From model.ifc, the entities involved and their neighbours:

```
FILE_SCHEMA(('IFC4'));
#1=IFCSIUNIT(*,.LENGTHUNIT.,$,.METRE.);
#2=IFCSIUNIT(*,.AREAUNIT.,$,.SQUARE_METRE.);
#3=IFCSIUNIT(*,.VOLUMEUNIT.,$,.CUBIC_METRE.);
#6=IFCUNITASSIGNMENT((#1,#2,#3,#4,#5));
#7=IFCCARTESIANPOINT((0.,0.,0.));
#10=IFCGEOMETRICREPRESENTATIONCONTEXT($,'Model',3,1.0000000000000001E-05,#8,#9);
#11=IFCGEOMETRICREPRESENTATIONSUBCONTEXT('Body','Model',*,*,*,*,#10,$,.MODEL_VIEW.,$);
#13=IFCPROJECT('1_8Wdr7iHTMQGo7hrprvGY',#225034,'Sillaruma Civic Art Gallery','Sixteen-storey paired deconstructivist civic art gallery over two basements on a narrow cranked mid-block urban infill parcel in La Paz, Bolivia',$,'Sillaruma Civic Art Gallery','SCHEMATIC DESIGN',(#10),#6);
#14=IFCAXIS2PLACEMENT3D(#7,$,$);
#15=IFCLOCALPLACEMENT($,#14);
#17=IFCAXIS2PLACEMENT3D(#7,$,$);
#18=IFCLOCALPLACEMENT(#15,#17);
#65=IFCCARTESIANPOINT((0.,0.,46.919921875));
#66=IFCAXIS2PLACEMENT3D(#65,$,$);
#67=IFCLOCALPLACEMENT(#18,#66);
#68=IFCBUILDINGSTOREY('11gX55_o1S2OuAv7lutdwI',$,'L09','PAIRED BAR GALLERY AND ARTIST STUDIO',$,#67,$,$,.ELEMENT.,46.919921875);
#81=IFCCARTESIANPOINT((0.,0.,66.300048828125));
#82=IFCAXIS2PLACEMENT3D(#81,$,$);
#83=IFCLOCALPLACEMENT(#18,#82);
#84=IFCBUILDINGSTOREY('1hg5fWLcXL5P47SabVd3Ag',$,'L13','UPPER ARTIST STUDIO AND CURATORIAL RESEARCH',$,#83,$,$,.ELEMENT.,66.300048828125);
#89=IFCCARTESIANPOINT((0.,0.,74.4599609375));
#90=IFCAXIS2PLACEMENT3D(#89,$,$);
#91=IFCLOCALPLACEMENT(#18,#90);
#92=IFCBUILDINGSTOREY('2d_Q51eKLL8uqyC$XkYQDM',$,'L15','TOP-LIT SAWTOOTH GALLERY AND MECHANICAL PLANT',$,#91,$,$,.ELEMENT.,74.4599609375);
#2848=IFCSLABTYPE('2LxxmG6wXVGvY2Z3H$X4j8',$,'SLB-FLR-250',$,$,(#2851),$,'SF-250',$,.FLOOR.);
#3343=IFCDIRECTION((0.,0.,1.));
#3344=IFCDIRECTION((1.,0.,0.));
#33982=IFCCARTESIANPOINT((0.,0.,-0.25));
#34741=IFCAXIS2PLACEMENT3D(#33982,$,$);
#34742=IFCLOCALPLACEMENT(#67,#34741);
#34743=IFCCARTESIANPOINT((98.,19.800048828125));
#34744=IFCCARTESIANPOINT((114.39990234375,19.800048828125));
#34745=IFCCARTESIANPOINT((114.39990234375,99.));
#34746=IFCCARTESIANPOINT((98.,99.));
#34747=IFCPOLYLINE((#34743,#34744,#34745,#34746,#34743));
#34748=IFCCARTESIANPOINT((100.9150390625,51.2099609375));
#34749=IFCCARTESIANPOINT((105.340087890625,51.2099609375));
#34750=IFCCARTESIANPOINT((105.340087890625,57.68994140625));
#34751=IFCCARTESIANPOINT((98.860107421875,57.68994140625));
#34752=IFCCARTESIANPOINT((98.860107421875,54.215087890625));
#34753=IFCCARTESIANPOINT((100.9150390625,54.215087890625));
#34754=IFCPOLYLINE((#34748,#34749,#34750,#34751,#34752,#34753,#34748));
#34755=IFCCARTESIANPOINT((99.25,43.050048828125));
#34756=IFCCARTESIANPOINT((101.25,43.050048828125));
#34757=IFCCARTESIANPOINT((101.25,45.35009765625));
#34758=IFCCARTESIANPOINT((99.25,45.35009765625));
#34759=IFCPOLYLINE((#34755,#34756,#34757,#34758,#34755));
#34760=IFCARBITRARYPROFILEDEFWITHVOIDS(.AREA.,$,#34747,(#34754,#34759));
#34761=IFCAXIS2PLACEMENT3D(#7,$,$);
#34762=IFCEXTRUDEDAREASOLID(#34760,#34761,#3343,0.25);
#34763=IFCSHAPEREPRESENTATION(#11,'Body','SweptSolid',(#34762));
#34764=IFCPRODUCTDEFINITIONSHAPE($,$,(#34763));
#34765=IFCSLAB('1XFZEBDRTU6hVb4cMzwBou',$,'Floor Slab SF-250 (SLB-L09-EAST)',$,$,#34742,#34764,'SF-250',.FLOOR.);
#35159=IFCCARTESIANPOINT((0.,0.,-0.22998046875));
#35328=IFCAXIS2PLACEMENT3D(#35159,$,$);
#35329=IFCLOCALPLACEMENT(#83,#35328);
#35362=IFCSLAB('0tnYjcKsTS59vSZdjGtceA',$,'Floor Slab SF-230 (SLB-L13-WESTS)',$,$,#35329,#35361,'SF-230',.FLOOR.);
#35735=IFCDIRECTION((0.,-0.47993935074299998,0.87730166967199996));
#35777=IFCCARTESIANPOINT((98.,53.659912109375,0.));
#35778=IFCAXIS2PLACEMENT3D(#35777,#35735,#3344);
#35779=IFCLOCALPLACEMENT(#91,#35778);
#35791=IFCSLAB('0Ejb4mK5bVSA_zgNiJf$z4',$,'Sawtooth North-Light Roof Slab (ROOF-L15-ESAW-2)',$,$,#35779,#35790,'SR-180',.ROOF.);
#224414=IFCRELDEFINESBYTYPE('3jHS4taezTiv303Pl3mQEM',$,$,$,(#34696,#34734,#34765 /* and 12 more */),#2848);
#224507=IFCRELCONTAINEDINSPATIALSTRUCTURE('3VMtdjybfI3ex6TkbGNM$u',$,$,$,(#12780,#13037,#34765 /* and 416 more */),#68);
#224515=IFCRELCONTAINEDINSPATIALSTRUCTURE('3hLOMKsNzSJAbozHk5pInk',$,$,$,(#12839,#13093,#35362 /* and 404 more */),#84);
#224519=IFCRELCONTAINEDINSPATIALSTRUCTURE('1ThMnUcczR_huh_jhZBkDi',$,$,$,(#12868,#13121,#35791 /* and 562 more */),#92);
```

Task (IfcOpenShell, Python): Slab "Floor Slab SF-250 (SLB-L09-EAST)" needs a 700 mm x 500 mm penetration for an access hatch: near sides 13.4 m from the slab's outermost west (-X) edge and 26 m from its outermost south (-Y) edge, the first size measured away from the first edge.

```python
import numpy as np
import ifcopenshell
import ifcopenshell.api.feature
import ifcopenshell.api.geometry
import ifcopenshell.api.root
import ifcopenshell.geom
import ifcopenshell.util.placement
import ifcopenshell.util.representation
import ifcopenshell.util.shape
import ifcopenshell.util.unit

model = ifcopenshell.open("model.ifc")
unit_scale = ifcopenshell.util.unit.calculate_unit_scale(model)
settings = ifcopenshell.geom.settings()


def volume(element):
    """Net volume in cubic metres, openings subtracted."""
    shape = ifcopenshell.geom.create_shape(settings, element)
    return ifcopenshell.util.shape.get_volume(shape.geometry)


slab = model.by_guid("1XFZEBDRTU6hVb4cMzwBou")
before = volume(slab)

# Extent in the slab's own axes, in metres. The edges named are its -X and -Y sides.
slab_shape = ifcopenshell.geom.create_shape(settings, slab)
vertices = ifcopenshell.util.shape.get_vertices(slab_shape.geometry)
x_min, y_min, bottom = vertices.min(axis=0)
top = vertices[:, 2].max()

opening = ifcopenshell.api.root.create_entity(model, ifc_class="IfcOpeningElement", name="Access hatch opening", predefined_type="OPENING")
context = ifcopenshell.util.representation.get_context(model, "Model", "Body", "MODEL_VIEW")
width, depth = 0.7, 0.5
outline = [(0.0, 0.0), (width, 0.0), (width, depth), (0.0, depth), (0.0, 0.0)]
# Overshoot both faces by 50 mm so the cut is clean.
shape = ifcopenshell.api.geometry.add_slab_representation(
    model, context=context, depth=top - bottom + 0.1, polyline=outline
)
ifcopenshell.api.geometry.assign_representation(model, product=opening, representation=shape)

matrix = ifcopenshell.util.placement.get_local_placement(slab.ObjectPlacement)
matrix[:, 3] = matrix @ np.append(np.array([x_min + 13.4, y_min + 26, bottom - 0.05]) / unit_scale, 1.0)
ifcopenshell.api.geometry.edit_object_placement(model, product=opening, matrix=matrix, is_si=False)
ifcopenshell.api.feature.add_feature(model, feature=opening, element=slab)

after = volume(slab)

print(f"slab volume {before:.3f} -> {after:.3f} m3")

model.write("model_edited.ifc")
```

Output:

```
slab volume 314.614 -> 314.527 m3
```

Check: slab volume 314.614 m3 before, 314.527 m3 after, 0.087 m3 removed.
